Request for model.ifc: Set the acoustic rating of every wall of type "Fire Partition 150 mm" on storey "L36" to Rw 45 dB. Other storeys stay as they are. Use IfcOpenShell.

First a look at what the model holds.

```python
import ifcopenshell
import ifcopenshell.util.element

model = ifcopenshell.open("model.ifc")
print(model.schema)
storey = next(s for s in model.by_type("IfcBuildingStorey") if s.Name == "L36")
walls = [e for e in ifcopenshell.util.element.get_decomposition(storey) if e.is_a("IfcWall")]
seen = {}
for e in walls:
    element_type = ifcopenshell.util.element.get_type(e)
    key = (element_type.Name if element_type != e and element_type else None, ifcopenshell.util.element.get_pset(e, "Pset_WallCommon", "AcousticRating"))
    seen[key] = seen.get(key, 0) + 1
for (name, value), count in sorted(seen.items(), key=str):
    print(count, "x", name, "|", value)
```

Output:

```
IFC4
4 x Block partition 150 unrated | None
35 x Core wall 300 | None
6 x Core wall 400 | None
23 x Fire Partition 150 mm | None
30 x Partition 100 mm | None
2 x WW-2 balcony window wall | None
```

```python
import ifcopenshell
import ifcopenshell.api.pset
import ifcopenshell.util.element

model = ifcopenshell.open("model.ifc")

storey = next(s for s in model.by_type("IfcBuildingStorey") if s.Name == "L36")
walls = [e for e in ifcopenshell.util.element.get_decomposition(storey) if e.is_a("IfcWall")]

count = 0
for e in walls:
    element_type = ifcopenshell.util.element.get_type(e)
    if element_type in (None, e) or element_type.Name != "Fire Partition 150 mm":
        continue
    found = ifcopenshell.util.element.get_pset(e, "Pset_WallCommon", should_inherit=False)
    if found:
        pset = model.by_id(found["id"])
        if len(ifcopenshell.util.element.get_elements_by_pset(pset)) > 1:
            pset = ifcopenshell.api.pset.unshare_pset(model, products=[e], pset=pset)[0]
    else:
        pset = ifcopenshell.api.pset.add_pset(model, product=e, name="Pset_WallCommon")
    ifcopenshell.api.pset.edit_pset(model, pset=pset, properties={"AcousticRating": "Rw 45 dB"})
    count += 1

print(count, "walls updated")

model.write("model-out.ifc")
```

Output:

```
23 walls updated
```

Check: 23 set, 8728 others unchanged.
